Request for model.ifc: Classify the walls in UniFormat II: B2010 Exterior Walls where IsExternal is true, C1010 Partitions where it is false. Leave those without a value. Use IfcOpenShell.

First a look at what the model holds.

```python
import ifcopenshell
import ifcopenshell.util.element

model = ifcopenshell.open("model.ifc")
print(model.schema)
print("classifications:", [c.Name for c in model.by_type("IfcClassification")])
values = [ifcopenshell.util.element.get_pset(e, "Pset_WallCommon", "IsExternal") for e in model.by_type("IfcWall")]
for value in (True, False, None):
    print("IsExternal", value, values.count(value))
```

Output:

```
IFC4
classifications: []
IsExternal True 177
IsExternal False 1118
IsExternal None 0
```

```python
import ifcopenshell
import ifcopenshell.api.classification
import ifcopenshell.util.element

model = ifcopenshell.open("model.ifc")

system = ifcopenshell.api.classification.add_classification(model, classification="UniFormat II")

walls = model.by_type("IfcWall")
external = {e: ifcopenshell.util.element.get_pset(e, "Pset_WallCommon", "IsExternal") for e in walls}
for flag, code, name in ((True, "B2010", "Exterior Walls"), (False, "C1010", "Partitions")):
    products = [e for e in walls if external[e] is flag]
    ifcopenshell.api.classification.add_reference(
        model, products=products, classification=system, identification=code, name=name
    )
    print(code, len(products))

model.write("model_edited.ifc")
```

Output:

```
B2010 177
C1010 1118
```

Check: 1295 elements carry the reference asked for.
